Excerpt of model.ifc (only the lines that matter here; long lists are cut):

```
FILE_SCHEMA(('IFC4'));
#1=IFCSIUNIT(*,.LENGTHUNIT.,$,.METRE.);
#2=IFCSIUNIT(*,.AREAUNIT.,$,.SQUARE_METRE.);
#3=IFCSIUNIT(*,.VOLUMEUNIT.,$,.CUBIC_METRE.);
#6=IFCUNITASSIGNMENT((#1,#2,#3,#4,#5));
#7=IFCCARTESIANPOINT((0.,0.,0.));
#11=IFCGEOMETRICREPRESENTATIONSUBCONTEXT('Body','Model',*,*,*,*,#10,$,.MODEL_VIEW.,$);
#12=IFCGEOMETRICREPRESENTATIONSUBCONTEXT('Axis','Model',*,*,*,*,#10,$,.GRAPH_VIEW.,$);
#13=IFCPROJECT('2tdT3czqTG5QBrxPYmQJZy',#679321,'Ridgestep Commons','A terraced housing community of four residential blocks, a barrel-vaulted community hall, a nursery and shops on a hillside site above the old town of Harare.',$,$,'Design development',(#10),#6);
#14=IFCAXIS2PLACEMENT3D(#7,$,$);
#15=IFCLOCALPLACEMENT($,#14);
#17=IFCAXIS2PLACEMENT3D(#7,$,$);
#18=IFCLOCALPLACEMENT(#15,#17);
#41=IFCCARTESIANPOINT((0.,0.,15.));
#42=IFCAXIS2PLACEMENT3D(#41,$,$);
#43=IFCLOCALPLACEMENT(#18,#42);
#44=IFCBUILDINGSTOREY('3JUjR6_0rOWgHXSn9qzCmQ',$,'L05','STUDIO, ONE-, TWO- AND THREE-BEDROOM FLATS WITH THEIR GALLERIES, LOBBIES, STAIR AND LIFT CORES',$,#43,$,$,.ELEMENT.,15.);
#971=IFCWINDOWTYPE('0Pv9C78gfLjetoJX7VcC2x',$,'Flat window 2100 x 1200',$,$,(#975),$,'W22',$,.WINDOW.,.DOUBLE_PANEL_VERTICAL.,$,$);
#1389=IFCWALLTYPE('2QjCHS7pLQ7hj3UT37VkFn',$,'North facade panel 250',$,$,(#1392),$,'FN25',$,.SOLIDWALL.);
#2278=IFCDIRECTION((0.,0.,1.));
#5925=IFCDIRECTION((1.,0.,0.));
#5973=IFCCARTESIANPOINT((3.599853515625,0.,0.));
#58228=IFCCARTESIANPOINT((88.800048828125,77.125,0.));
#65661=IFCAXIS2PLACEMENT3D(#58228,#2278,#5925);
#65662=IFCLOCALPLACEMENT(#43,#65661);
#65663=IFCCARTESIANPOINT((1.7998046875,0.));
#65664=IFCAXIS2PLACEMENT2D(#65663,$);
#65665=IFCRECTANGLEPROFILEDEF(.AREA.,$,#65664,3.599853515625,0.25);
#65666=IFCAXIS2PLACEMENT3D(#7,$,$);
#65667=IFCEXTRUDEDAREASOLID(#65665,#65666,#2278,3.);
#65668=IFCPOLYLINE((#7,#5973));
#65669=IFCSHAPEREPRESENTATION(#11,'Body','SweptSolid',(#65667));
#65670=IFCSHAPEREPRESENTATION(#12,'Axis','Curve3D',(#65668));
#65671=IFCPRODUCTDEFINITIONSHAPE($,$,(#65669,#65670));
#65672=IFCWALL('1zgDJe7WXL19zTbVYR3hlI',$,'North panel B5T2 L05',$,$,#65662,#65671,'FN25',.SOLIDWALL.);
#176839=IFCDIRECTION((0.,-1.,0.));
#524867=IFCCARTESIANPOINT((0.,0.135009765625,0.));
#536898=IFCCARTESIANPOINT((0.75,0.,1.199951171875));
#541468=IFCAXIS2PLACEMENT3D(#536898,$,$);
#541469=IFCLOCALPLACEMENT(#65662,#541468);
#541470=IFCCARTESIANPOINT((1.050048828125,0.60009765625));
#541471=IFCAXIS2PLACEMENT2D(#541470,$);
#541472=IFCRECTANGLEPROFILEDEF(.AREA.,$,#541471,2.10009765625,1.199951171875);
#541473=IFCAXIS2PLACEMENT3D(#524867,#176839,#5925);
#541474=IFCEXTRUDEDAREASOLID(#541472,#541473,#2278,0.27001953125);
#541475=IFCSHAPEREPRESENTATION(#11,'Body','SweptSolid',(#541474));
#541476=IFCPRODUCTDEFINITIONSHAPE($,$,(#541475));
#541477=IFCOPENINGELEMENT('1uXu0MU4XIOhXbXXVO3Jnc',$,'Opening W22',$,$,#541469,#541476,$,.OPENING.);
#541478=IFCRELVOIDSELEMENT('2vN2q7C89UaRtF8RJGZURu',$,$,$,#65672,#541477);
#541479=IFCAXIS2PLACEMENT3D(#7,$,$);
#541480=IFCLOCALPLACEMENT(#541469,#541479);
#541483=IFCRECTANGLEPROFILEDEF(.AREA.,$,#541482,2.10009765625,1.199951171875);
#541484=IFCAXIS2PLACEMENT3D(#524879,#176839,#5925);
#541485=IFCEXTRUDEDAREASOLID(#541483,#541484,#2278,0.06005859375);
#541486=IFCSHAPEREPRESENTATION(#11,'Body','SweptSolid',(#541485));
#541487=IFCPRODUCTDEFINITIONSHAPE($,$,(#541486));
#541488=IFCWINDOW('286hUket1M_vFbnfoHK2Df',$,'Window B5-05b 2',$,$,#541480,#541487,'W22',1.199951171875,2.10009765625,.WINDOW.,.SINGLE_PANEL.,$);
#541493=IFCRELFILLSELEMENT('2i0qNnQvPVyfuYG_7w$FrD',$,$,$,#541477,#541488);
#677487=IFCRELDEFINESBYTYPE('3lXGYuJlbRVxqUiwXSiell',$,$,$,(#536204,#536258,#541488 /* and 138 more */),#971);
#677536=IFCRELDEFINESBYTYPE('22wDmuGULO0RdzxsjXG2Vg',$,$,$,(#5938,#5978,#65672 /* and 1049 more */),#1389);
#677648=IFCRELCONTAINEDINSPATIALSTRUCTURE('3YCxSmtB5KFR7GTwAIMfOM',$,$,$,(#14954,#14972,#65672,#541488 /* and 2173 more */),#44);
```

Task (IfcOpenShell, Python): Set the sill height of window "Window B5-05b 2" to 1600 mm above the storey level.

```python
import numpy as np
import ifcopenshell
import ifcopenshell.api.geometry
import ifcopenshell.geom
import ifcopenshell.util.element
import ifcopenshell.util.placement
import ifcopenshell.util.shape
import ifcopenshell.util.unit

model = ifcopenshell.open("model.ifc")
unit_scale = ifcopenshell.util.unit.calculate_unit_scale(model)

window = model.by_guid("286hUket1M_vFbnfoHK2Df")
opening = window.FillsVoids[0].RelatingOpeningElement
storey = ifcopenshell.util.element.get_container(window, ifc_class="IfcBuildingStorey")
level = ifcopenshell.util.placement.get_local_placement(storey.ObjectPlacement)[2, 3]

# The opening's origin need not be at the sill, so measure its lowest point.
shape = ifcopenshell.geom.create_shape(ifcopenshell.geom.settings(), opening)
bottom = ifcopenshell.util.shape.get_shape_bottom_elevation(shape, shape.geometry) / unit_scale
dz = level + 1.6 / unit_scale - bottom

shift = np.array([0.0, 0.0, dz])
# The window is placed relative to its opening, so it follows when the opening moves.
matrix = ifcopenshell.util.placement.get_local_placement(opening.ObjectPlacement)
matrix[:3, 3] += shift
ifcopenshell.api.geometry.edit_object_placement(
    model, product=opening, matrix=matrix, is_si=False, should_transform_children=True
)

print(f"moved by {dz * unit_scale:+.3f} m")

model.write("model_edited.ifc")
```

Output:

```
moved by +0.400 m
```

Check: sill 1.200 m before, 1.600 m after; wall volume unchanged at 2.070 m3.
